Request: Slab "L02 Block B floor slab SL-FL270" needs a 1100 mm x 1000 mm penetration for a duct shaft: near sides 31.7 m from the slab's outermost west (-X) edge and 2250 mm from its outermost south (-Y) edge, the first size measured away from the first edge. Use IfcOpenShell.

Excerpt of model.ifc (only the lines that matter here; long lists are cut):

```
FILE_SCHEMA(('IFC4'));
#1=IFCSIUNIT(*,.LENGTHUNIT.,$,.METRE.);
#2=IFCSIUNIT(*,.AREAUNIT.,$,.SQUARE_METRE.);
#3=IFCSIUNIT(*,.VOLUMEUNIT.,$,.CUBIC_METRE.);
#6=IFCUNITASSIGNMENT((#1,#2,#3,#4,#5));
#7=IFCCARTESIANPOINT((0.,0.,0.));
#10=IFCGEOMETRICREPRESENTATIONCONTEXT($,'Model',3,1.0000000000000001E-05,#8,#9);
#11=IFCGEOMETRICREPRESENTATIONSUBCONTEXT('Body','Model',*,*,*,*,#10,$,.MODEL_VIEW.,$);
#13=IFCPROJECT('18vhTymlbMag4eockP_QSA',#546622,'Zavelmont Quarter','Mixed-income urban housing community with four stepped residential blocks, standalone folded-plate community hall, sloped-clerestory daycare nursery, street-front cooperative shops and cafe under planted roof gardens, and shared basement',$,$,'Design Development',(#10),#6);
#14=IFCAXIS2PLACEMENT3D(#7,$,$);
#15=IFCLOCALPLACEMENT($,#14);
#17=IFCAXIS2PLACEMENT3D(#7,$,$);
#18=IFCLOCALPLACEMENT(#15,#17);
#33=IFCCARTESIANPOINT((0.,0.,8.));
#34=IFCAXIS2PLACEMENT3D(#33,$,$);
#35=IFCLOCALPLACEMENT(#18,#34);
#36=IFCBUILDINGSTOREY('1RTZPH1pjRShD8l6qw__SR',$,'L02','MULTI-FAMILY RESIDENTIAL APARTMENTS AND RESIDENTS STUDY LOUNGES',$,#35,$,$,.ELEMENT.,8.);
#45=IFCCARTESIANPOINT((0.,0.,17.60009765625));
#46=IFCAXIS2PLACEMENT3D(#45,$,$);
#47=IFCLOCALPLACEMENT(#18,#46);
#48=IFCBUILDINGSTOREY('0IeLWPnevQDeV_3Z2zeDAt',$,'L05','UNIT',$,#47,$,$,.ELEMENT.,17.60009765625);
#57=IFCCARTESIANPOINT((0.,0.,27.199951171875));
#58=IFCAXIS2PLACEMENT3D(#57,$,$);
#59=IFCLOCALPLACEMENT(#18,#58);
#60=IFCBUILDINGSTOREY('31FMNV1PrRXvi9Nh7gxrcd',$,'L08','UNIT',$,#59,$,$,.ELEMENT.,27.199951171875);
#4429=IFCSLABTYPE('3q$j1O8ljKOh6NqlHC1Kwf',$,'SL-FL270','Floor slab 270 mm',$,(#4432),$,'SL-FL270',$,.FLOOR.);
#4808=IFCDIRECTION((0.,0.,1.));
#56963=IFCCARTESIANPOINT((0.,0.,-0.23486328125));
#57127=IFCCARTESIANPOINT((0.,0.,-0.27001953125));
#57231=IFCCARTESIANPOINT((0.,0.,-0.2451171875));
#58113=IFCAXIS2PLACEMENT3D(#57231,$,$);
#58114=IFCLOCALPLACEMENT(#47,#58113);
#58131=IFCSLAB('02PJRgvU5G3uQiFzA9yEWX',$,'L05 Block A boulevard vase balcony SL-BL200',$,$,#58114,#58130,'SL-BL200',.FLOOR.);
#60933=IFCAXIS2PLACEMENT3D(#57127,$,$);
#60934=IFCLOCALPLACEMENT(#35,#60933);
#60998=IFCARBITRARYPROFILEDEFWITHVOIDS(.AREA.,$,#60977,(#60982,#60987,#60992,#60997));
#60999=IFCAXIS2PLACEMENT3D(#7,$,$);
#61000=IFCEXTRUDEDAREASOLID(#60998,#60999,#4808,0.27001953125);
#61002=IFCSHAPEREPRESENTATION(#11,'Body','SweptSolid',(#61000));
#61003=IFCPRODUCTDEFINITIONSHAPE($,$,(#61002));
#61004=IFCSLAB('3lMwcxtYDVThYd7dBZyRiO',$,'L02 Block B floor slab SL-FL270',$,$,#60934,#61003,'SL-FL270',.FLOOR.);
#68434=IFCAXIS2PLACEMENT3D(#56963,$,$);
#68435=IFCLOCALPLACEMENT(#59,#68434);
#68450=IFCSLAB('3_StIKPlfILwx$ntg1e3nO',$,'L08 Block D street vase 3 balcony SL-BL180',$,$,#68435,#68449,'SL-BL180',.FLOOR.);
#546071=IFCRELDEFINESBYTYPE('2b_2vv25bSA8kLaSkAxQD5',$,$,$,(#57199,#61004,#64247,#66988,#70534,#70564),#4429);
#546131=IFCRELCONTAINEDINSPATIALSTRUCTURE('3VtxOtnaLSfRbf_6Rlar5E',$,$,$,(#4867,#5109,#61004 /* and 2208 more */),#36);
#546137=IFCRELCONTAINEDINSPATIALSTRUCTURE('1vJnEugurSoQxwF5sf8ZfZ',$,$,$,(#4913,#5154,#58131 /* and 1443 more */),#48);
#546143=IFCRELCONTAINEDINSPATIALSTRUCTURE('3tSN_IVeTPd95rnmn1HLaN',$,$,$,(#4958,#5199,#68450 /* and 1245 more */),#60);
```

```python
import numpy as np
import ifcopenshell
import ifcopenshell.api.feature
import ifcopenshell.api.geometry
import ifcopenshell.api.root
import ifcopenshell.geom
import ifcopenshell.util.placement
import ifcopenshell.util.representation
import ifcopenshell.util.shape
import ifcopenshell.util.unit

model = ifcopenshell.open("model.ifc")
unit_scale = ifcopenshell.util.unit.calculate_unit_scale(model)
settings = ifcopenshell.geom.settings()


def volume(element):
    """Net volume in cubic metres, openings subtracted."""
    shape = ifcopenshell.geom.create_shape(settings, element)
    return ifcopenshell.util.shape.get_volume(shape.geometry)


slab = model.by_guid("3lMwcxtYDVThYd7dBZyRiO")
before = volume(slab)

# Extent in the slab's own axes, in metres. The edges named are its -X and -Y sides.
slab_shape = ifcopenshell.geom.create_shape(settings, slab)
vertices = ifcopenshell.util.shape.get_vertices(slab_shape.geometry)
x_min, y_min, bottom = vertices.min(axis=0)
top = vertices[:, 2].max()

opening = ifcopenshell.api.root.create_entity(model, ifc_class="IfcOpeningElement", name="Duct shaft opening", predefined_type="OPENING")
context = ifcopenshell.util.representation.get_context(model, "Model", "Body", "MODEL_VIEW")
width, depth = 1.1, 1
outline = [(0.0, 0.0), (width, 0.0), (width, depth), (0.0, depth), (0.0, 0.0)]
# Overshoot both faces by 50 mm so the cut is clean.
shape = ifcopenshell.api.geometry.add_slab_representation(
    model, context=context, depth=top - bottom + 0.1, polyline=outline
)
ifcopenshell.api.geometry.assign_representation(model, product=opening, representation=shape)

matrix = ifcopenshell.util.placement.get_local_placement(slab.ObjectPlacement)
matrix[:, 3] = matrix @ np.append(np.array([x_min + 31.7, y_min + 2.25, bottom - 0.05]) / unit_scale, 1.0)
ifcopenshell.api.geometry.edit_object_placement(model, product=opening, matrix=matrix, is_si=False)
ifcopenshell.api.feature.add_feature(model, feature=opening, element=slab)

after = volume(slab)

print(f"slab volume {before:.3f} -> {after:.3f} m3")

model.write("model_updated.ifc")
```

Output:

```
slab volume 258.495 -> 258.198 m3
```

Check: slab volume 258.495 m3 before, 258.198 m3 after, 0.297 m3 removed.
